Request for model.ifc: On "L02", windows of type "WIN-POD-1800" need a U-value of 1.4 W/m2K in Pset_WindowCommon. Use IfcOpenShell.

First a look at what the model holds.

```python
import ifcopenshell
import ifcopenshell.util.element

model = ifcopenshell.open("model.ifc")
print(model.schema)
storey = next(s for s in model.by_type("IfcBuildingStorey") if s.Name == "L02")
windows = [e for e in ifcopenshell.util.element.get_decomposition(storey) if e.is_a("IfcWindow")]
seen = {}
for e in windows:
    element_type = ifcopenshell.util.element.get_type(e)
    key = (element_type.Name if element_type != e and element_type else None, ifcopenshell.util.element.get_pset(e, "Pset_WindowCommon", "ThermalTransmittance"))
    seen[key] = seen.get(key, 0) + 1
for (name, value), count in sorted(seen.items(), key=str):
    print(count, "x", name, "|", value)
```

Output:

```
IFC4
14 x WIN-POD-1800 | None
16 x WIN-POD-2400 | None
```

```python
import ifcopenshell
import ifcopenshell.api.pset
import ifcopenshell.util.element

model = ifcopenshell.open("model.ifc")

storey = next(s for s in model.by_type("IfcBuildingStorey") if s.Name == "L02")
windows = [e for e in ifcopenshell.util.element.get_decomposition(storey) if e.is_a("IfcWindow")]

count = 0
for e in windows:
    element_type = ifcopenshell.util.element.get_type(e)
    if element_type in (None, e) or element_type.Name != "WIN-POD-1800":
        continue
    # add_pset returns the element's existing set when there is one.
    pset = ifcopenshell.api.pset.add_pset(model, product=e, name="Pset_WindowCommon")
    ifcopenshell.api.pset.edit_pset(model, pset=pset, properties={"ThermalTransmittance": 1.4})
    count += 1

print(count, "windows updated")

model.write("model_updated.ifc")
```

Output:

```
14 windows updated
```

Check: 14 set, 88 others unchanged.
